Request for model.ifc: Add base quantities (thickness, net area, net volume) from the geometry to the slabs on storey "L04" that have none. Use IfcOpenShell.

First a look at what the model holds.

```python
import ifcopenshell
import ifcopenshell.util.element
import ifcopenshell.util.unit

model = ifcopenshell.open("model.ifc")
print(model.schema)
for unit_type in ("LENGTHUNIT", "AREAUNIT", "VOLUMEUNIT"):
    print(unit_type, ifcopenshell.util.unit.calculate_unit_scale(model, unit_type))
storey = next(s for s in model.by_type("IfcBuildingStorey") if s.Name == "L04")
slabs = [e for e in ifcopenshell.util.element.get_decomposition(storey) if e.is_a("IfcSlab")]
for e in sorted(slabs, key=lambda e: e.id()):
    print(e.id(), e.is_a(), e.Name, list(ifcopenshell.util.element.get_psets(e, qtos_only=True)), sep=" | ")
```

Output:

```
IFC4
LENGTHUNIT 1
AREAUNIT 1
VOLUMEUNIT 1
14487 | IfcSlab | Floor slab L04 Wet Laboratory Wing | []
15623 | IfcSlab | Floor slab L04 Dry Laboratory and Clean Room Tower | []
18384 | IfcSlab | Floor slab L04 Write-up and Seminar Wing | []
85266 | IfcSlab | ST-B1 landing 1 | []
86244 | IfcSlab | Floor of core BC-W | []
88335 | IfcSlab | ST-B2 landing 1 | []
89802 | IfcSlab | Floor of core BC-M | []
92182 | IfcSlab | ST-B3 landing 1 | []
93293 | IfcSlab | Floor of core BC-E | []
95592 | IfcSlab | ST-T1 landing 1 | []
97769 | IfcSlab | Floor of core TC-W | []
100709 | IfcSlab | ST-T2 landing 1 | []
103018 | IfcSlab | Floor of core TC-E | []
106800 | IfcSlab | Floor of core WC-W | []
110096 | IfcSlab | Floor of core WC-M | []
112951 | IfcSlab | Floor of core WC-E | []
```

```python
import ifcopenshell
import ifcopenshell.api.pset
import ifcopenshell.geom
import ifcopenshell.util.element
import ifcopenshell.util.shape
import ifcopenshell.util.unit

model = ifcopenshell.open("model.ifc")
unit_scale = ifcopenshell.util.unit.calculate_unit_scale(model)
area_scale = ifcopenshell.util.unit.calculate_unit_scale(model, "AREAUNIT")
volume_scale = ifcopenshell.util.unit.calculate_unit_scale(model, "VOLUMEUNIT")
settings = ifcopenshell.geom.settings()

storey = next(s for s in model.by_type("IfcBuildingStorey") if s.Name == "L04")
slabs = [e for e in ifcopenshell.util.element.get_decomposition(storey) if e.is_a("IfcSlab")]

for e in sorted(slabs, key=lambda e: e.id()):
    if ifcopenshell.util.element.get_psets(e, qtos_only=True, should_inherit=False):
        continue
    # Geometry comes back in metres, in the element's own axes.
    shape = ifcopenshell.geom.create_shape(settings, e)
    values = {
        "Width": ifcopenshell.util.shape.get_z(shape.geometry) / unit_scale,
        "NetArea": ifcopenshell.util.shape.get_footprint_area(shape.geometry) / area_scale,
        "NetVolume": ifcopenshell.util.shape.get_volume(shape.geometry) / volume_scale,
    }
    qto = ifcopenshell.api.pset.add_qto(model, product=e, name="Qto_SlabBaseQuantities")
    ifcopenshell.api.pset.edit_qto(model, qto=qto, properties=values)
    print(e.id(), {k: round(v, 3) for k, v in values.items()})

model.write("model-out.ifc")
```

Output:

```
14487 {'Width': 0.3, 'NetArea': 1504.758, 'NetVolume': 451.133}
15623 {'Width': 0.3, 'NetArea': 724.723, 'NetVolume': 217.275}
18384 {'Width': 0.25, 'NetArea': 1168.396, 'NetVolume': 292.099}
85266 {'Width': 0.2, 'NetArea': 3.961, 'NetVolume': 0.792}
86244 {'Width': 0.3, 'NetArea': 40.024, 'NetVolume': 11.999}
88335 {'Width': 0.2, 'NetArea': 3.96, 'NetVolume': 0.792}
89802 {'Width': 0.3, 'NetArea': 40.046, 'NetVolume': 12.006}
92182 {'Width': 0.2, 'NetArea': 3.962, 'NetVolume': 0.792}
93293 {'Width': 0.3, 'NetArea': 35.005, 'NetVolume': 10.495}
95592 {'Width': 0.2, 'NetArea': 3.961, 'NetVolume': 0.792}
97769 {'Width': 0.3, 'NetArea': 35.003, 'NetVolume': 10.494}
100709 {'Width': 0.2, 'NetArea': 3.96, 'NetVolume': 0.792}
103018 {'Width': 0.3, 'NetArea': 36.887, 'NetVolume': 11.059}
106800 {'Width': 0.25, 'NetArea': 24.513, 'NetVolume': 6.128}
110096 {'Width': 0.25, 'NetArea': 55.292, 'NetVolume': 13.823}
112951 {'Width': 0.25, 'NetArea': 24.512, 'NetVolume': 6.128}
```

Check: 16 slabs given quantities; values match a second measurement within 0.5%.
